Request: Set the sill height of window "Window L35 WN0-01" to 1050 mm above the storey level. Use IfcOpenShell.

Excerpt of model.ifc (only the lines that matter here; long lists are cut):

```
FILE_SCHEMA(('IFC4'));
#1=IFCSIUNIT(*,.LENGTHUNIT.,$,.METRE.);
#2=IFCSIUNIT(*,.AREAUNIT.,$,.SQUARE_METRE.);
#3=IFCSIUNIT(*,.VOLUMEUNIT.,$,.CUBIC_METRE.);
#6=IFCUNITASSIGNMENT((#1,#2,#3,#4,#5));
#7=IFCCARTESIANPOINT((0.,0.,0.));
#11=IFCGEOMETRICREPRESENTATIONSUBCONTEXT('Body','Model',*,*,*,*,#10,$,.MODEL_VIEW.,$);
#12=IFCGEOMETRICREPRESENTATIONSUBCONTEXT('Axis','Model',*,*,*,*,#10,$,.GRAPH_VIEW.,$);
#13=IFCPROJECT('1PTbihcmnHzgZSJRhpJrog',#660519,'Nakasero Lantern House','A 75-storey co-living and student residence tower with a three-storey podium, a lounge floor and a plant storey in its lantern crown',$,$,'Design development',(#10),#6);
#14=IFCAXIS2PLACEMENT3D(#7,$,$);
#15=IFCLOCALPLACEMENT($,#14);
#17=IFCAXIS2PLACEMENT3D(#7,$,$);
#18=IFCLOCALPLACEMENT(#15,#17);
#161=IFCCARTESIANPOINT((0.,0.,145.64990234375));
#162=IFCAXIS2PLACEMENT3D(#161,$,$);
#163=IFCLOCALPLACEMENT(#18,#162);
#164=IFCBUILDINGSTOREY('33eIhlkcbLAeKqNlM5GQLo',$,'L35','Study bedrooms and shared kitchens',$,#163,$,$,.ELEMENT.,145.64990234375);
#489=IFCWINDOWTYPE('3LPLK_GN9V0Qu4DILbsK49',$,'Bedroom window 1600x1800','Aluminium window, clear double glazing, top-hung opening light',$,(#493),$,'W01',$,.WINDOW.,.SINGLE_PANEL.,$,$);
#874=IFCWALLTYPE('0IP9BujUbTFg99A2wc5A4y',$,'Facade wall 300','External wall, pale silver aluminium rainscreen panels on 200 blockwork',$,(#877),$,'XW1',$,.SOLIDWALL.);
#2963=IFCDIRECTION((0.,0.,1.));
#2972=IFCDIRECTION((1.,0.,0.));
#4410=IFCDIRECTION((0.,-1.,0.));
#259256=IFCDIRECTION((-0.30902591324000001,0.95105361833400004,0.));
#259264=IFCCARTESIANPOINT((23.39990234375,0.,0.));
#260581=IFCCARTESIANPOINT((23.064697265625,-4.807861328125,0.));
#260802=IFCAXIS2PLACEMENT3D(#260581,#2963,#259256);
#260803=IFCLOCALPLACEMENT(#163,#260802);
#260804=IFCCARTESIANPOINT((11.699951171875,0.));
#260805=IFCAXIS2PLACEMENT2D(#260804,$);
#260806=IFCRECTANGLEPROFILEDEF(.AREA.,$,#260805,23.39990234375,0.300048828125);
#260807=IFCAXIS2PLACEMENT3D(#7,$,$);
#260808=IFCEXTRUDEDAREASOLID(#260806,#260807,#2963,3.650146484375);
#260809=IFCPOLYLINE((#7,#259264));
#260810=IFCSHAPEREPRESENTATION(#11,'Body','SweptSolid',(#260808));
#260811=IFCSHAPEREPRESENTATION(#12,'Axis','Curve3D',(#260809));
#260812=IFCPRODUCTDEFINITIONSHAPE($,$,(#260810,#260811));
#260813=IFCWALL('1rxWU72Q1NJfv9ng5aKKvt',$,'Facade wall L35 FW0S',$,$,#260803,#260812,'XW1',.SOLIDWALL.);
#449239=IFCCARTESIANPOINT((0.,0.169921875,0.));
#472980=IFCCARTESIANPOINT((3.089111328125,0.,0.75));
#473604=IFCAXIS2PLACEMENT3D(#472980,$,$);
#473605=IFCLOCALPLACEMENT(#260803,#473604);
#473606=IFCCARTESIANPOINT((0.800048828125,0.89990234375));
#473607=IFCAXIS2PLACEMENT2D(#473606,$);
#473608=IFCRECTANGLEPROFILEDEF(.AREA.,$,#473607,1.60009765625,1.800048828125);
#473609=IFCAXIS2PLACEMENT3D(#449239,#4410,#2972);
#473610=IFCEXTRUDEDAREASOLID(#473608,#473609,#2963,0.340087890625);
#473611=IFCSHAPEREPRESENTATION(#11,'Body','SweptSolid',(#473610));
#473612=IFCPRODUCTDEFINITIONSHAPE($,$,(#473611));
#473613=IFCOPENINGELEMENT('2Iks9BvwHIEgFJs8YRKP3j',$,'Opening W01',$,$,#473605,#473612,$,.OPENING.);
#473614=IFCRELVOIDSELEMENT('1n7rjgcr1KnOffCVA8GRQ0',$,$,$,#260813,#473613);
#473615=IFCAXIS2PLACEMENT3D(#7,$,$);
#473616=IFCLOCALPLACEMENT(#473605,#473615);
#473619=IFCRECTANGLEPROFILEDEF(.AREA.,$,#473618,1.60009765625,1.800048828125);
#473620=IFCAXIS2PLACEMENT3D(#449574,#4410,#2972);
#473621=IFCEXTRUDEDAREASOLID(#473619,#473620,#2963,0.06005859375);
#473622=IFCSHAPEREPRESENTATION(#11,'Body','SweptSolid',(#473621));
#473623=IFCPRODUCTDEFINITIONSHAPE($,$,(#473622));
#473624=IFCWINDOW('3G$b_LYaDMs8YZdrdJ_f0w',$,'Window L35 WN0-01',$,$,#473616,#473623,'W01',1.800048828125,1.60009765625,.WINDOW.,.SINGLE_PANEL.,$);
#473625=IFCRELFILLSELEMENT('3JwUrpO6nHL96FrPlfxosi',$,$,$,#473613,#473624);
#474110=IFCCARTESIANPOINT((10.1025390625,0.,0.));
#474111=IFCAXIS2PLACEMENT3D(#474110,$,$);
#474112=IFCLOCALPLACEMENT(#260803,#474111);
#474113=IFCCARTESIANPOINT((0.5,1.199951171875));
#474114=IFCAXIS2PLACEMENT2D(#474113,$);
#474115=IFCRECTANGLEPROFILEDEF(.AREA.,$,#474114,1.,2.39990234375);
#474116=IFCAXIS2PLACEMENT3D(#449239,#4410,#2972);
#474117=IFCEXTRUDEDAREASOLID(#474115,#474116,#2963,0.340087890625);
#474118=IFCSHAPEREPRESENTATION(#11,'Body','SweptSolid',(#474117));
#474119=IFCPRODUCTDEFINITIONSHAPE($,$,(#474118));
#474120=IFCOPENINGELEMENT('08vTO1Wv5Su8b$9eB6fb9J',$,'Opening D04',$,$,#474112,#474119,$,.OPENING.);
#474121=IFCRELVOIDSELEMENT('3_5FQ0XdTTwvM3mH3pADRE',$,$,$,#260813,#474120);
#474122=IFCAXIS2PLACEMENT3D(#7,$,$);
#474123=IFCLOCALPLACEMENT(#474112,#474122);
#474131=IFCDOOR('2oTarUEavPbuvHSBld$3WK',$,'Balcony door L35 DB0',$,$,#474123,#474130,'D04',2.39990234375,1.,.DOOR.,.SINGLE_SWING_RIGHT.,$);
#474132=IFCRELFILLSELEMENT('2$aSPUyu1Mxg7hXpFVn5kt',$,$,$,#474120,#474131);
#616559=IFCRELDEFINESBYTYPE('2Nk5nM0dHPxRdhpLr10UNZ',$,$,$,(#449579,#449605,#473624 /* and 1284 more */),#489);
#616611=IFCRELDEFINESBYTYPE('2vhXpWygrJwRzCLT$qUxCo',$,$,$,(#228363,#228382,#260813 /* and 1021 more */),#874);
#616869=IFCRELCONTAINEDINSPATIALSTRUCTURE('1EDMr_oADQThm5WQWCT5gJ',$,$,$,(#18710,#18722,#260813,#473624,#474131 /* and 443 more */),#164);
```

```python
import numpy as np
import ifcopenshell
import ifcopenshell.api.geometry
import ifcopenshell.geom
import ifcopenshell.util.element
import ifcopenshell.util.placement
import ifcopenshell.util.shape
import ifcopenshell.util.unit

model = ifcopenshell.open("model.ifc")
unit_scale = ifcopenshell.util.unit.calculate_unit_scale(model)

window = model.by_id(473624)
opening = window.FillsVoids[0].RelatingOpeningElement
storey = ifcopenshell.util.element.get_container(window, ifc_class="IfcBuildingStorey")
level = ifcopenshell.util.placement.get_local_placement(storey.ObjectPlacement)[2, 3]

# The opening's origin need not be at the sill, so measure its lowest point.
shape = ifcopenshell.geom.create_shape(ifcopenshell.geom.settings(), opening)
bottom = ifcopenshell.util.shape.get_shape_bottom_elevation(shape, shape.geometry) / unit_scale
dz = level + 1.05 / unit_scale - bottom

shift = np.array([0.0, 0.0, dz])
# The window is placed relative to its opening, so it follows when the opening moves.
matrix = ifcopenshell.util.placement.get_local_placement(opening.ObjectPlacement)
matrix[:3, 3] += shift
ifcopenshell.api.geometry.edit_object_placement(
    model, product=opening, matrix=matrix, is_si=False, should_transform_children=True
)

print(f"moved by {dz * unit_scale:+.3f} m")

model.write("model_updated.ifc")
```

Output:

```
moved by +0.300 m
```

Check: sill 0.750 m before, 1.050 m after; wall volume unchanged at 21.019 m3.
